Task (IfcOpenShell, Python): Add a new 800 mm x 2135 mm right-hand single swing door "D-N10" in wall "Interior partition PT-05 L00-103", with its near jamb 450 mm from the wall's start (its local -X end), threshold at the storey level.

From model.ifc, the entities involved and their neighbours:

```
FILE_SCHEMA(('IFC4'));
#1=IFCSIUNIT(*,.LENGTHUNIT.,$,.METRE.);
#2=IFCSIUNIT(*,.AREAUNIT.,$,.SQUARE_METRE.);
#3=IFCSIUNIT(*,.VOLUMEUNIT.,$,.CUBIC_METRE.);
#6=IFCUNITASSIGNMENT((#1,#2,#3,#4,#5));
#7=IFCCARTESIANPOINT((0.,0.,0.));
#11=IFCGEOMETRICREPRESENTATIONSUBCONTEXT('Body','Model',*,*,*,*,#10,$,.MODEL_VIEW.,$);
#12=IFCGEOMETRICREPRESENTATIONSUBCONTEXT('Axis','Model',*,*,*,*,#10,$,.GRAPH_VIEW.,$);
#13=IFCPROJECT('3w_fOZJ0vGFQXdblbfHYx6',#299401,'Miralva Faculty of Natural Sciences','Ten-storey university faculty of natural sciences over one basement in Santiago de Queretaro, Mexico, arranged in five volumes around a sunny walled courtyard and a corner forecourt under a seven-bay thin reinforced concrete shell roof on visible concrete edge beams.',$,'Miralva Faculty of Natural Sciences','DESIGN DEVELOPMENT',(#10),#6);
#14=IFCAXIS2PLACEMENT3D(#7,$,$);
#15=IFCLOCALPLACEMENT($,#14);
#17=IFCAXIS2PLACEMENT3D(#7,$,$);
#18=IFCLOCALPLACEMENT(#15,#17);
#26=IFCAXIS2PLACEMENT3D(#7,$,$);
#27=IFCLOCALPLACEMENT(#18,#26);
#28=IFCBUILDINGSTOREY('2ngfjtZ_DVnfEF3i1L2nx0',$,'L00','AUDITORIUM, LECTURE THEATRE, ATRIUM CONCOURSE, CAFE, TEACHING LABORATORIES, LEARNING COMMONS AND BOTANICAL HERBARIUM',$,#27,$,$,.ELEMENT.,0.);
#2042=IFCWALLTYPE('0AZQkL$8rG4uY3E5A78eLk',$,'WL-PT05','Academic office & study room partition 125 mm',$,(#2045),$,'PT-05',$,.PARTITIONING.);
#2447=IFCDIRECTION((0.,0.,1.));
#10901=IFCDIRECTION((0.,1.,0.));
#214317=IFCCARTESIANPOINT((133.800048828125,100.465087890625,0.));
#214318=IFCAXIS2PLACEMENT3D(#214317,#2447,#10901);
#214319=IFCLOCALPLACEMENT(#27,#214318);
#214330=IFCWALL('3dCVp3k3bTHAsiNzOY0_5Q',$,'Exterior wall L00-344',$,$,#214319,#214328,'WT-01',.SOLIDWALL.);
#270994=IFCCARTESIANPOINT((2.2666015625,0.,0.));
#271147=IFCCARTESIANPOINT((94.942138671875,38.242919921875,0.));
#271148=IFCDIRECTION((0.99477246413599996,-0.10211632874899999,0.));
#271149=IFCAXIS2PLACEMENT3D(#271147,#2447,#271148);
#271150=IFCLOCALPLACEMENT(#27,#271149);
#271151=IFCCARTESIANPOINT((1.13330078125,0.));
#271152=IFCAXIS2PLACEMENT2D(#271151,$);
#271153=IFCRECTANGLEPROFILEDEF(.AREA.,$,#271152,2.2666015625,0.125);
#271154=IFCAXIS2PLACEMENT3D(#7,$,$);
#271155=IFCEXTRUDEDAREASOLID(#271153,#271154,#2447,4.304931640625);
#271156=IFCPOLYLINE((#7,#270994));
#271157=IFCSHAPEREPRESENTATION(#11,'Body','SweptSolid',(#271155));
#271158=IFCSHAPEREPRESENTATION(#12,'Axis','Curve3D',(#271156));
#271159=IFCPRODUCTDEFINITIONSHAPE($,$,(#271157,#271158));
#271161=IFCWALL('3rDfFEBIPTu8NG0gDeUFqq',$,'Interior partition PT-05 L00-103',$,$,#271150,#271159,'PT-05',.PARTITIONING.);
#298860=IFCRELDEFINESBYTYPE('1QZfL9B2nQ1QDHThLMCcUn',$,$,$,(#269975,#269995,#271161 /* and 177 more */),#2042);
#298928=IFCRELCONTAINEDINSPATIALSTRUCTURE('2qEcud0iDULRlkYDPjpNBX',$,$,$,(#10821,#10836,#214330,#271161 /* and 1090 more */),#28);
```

```python
import numpy as np
import ifcopenshell
import ifcopenshell.api.feature
import ifcopenshell.api.geometry
import ifcopenshell.api.root
import ifcopenshell.api.spatial
import ifcopenshell.geom
import ifcopenshell.util.element
import ifcopenshell.util.placement
import ifcopenshell.util.representation
import ifcopenshell.util.shape
import ifcopenshell.util.unit

model = ifcopenshell.open("model.ifc")
unit_scale = ifcopenshell.util.unit.calculate_unit_scale(model)
settings = ifcopenshell.geom.settings()


def volume(element):
    """Net volume in cubic metres, openings subtracted."""
    shape = ifcopenshell.geom.create_shape(settings, element)
    return ifcopenshell.util.shape.get_volume(shape.geometry)


wall = model.by_id(271161)
storey = ifcopenshell.util.element.get_container(wall, ifc_class="IfcBuildingStorey")
context = ifcopenshell.util.representation.get_context(model, "Model", "Body", "MODEL_VIEW")
before = volume(wall)

width, height, from_end, sill = 0.8, 2.135, 0.45, 0.0  # metres

# The wall runs along its own X axis, and the end named is its -X end.
wall_shape = ifcopenshell.geom.create_shape(settings, wall)
x, y, z = ifcopenshell.util.shape.get_vertices(wall_shape.geometry).T
start = x.min() + from_end
face, thickness = float(y.min()), float(y.max() - y.min())
wall_matrix = ifcopenshell.util.placement.get_local_placement(wall.ObjectPlacement)
level = ifcopenshell.util.placement.get_local_placement(storey.ObjectPlacement)[2, 3]


def in_wall(x, y):
    """Placement at x, y metres in the wall's axes, at sill height."""
    matrix = wall_matrix.copy()
    matrix[:, 3] = wall_matrix @ np.array([x / unit_scale, y / unit_scale, 0.0, 1.0])
    matrix[2, 3] = level + sill / unit_scale
    return matrix


# Opening: a box that overshoots both wall faces by 50 mm.
opening = ifcopenshell.api.root.create_entity(model, ifc_class="IfcOpeningElement", predefined_type="OPENING")
box = ifcopenshell.api.geometry.add_wall_representation(
    model, context=context, length=width, height=height, thickness=thickness + 0.1
)
ifcopenshell.api.geometry.assign_representation(model, product=opening, representation=box)
ifcopenshell.api.geometry.edit_object_placement(model, product=opening, matrix=in_wall(start, face - 0.05), is_si=False)
ifcopenshell.api.feature.add_feature(model, feature=opening, element=wall)

door = ifcopenshell.api.root.create_entity(model, ifc_class="IfcDoor", name="D-N10", predefined_type="DOOR")
door.OverallWidth, door.OverallHeight = width / unit_scale, height / unit_scale
door.OperationType = "SINGLE_SWING_RIGHT"
body = ifcopenshell.api.geometry.add_door_representation(
    model,
    context=context,
    overall_width=door.OverallWidth,
    overall_height=door.OverallHeight,
    operation_type="SINGLE_SWING_RIGHT",
    lining_properties={"LiningDepth": thickness / unit_scale, "ThresholdDepth": thickness / unit_scale},
)
ifcopenshell.api.geometry.assign_representation(model, product=door, representation=body)
ifcopenshell.api.spatial.assign_container(model, products=[door], relating_structure=storey)
ifcopenshell.api.feature.add_filling(model, opening=opening, element=door)

# The lining spans the wall, so the door starts at the wall face.
ifcopenshell.api.geometry.edit_object_placement(model, product=door, matrix=in_wall(start, face), is_si=False)

after = volume(wall)

print(f"wall volume {before:.3f} -> {after:.3f} m3")

model.write("model_edited.ifc")
```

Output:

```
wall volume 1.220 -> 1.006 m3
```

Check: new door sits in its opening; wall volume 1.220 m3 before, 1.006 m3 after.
